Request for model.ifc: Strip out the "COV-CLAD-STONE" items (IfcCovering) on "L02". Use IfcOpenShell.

First a look at what the model holds.

```python
import ifcopenshell
import ifcopenshell.util.element

model = ifcopenshell.open("model.ifc")
print(model.schema)
storey = next(s for s in model.by_type("IfcBuildingStorey") if s.Name == "L02")
coverings = [e for e in ifcopenshell.util.element.get_decomposition(storey) if e.is_a("IfcCovering")]
seen = {}
for e in coverings:
    element_type = ifcopenshell.util.element.get_type(e)
    name = element_type.Name if element_type not in (None, e) else None
    seen[name] = seen.get(name, 0) + 1
for name, count in sorted(seen.items(), key=str):
    print(count, "x", name)
```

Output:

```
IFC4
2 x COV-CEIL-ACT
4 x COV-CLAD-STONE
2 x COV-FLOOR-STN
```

```python
import ifcopenshell
import ifcopenshell.api.root
import ifcopenshell.util.element

model = ifcopenshell.open("model.ifc")

storey = next(s for s in model.by_type("IfcBuildingStorey") if s.Name == "L02")
coverings = [e for e in ifcopenshell.util.element.get_decomposition(storey) if e.is_a("IfcCovering")]
targets = [e for e in coverings if (t := ifcopenshell.util.element.get_type(e)) not in (None, e) and t.Name == "COV-CLAD-STONE"]

for e in targets:
    ifcopenshell.api.root.remove_product(model, product=e)
print(len(targets), "removed")

model.write("model-out.ifc")
```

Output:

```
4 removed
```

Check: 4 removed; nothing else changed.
